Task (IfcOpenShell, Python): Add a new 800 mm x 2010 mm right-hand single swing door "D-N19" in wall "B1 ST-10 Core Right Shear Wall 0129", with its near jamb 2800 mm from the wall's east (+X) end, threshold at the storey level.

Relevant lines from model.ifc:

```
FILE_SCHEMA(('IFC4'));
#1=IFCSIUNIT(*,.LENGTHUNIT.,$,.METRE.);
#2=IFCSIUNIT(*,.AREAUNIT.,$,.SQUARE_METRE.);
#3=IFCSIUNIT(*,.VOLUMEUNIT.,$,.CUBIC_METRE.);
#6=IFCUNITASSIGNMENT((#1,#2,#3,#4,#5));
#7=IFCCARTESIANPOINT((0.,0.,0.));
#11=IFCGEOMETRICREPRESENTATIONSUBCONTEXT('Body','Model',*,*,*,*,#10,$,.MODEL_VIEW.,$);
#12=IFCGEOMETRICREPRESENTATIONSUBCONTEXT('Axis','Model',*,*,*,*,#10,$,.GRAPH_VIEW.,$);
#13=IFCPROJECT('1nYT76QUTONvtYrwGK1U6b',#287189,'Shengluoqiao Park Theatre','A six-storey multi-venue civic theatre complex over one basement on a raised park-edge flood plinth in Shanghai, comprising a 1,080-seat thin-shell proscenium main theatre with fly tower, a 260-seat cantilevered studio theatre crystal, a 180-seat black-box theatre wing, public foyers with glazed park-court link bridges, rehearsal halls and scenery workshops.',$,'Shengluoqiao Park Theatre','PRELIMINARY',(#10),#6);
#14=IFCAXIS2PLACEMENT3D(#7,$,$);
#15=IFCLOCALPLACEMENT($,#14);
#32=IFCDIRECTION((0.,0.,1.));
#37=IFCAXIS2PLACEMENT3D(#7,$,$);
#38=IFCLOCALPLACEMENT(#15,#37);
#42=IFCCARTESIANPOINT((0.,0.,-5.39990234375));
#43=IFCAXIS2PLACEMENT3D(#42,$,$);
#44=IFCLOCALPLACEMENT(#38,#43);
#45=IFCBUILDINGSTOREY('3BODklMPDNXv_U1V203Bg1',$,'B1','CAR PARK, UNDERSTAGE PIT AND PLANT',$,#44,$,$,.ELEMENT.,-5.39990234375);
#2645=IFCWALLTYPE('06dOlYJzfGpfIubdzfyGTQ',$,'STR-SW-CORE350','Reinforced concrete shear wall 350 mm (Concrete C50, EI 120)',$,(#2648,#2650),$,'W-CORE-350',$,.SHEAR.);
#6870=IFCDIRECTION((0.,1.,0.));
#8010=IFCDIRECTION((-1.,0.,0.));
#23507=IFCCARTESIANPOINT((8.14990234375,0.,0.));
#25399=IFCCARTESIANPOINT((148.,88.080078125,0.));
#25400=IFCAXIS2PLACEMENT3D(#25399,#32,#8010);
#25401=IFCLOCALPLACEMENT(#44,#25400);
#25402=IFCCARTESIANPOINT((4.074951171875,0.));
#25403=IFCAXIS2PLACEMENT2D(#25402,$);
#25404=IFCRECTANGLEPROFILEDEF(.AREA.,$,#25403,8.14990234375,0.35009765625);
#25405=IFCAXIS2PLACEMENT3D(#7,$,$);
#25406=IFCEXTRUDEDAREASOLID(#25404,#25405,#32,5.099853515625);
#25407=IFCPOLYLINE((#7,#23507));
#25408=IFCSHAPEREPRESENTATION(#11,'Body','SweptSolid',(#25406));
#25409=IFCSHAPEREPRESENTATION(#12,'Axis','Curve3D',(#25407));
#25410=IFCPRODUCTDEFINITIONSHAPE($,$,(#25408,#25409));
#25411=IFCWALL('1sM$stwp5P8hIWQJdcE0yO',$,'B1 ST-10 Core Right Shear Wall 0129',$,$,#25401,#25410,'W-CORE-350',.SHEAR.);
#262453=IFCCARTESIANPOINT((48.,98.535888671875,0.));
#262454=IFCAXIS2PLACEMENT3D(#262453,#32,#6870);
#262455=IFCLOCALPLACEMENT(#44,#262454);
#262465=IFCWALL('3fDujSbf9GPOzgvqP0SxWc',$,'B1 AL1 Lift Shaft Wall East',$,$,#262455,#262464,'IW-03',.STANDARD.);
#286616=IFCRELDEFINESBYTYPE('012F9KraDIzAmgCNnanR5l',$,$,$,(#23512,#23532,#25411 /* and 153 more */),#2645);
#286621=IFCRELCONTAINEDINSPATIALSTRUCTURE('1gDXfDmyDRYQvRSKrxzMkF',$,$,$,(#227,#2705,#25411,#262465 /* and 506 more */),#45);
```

```python
import numpy as np
import ifcopenshell
import ifcopenshell.api.feature
import ifcopenshell.api.geometry
import ifcopenshell.api.root
import ifcopenshell.api.spatial
import ifcopenshell.geom
import ifcopenshell.util.element
import ifcopenshell.util.placement
import ifcopenshell.util.representation
import ifcopenshell.util.shape
import ifcopenshell.util.unit

model = ifcopenshell.open("model.ifc")
unit_scale = ifcopenshell.util.unit.calculate_unit_scale(model)
settings = ifcopenshell.geom.settings()


def volume(element):
    """Net volume in cubic metres, openings subtracted."""
    shape = ifcopenshell.geom.create_shape(settings, element)
    return ifcopenshell.util.shape.get_volume(shape.geometry)


wall = model.by_guid("1sM$stwp5P8hIWQJdcE0yO")
storey = ifcopenshell.util.element.get_container(wall, ifc_class="IfcBuildingStorey")
context = ifcopenshell.util.representation.get_context(model, "Model", "Body", "MODEL_VIEW")
before = volume(wall)

width, height, from_end, sill = 0.8, 2.01, 2.8, 0.0  # metres

# The wall runs along its own X axis, and the end named is its -X end.
wall_shape = ifcopenshell.geom.create_shape(settings, wall)
x, y, z = ifcopenshell.util.shape.get_vertices(wall_shape.geometry).T
start = x.min() + from_end
face, thickness = float(y.min()), float(y.max() - y.min())
wall_matrix = ifcopenshell.util.placement.get_local_placement(wall.ObjectPlacement)
level = ifcopenshell.util.placement.get_local_placement(storey.ObjectPlacement)[2, 3]


def in_wall(x, y):
    """Placement at x, y metres in the wall's axes, at sill height."""
    matrix = wall_matrix.copy()
    matrix[:, 3] = wall_matrix @ np.array([x / unit_scale, y / unit_scale, 0.0, 1.0])
    matrix[2, 3] = level + sill / unit_scale
    return matrix


# Opening: a box that overshoots both wall faces by 50 mm.
opening = ifcopenshell.api.root.create_entity(model, ifc_class="IfcOpeningElement", predefined_type="OPENING")
box = ifcopenshell.api.geometry.add_wall_representation(
    model, context=context, length=width, height=height, thickness=thickness + 0.1
)
ifcopenshell.api.geometry.assign_representation(model, product=opening, representation=box)
ifcopenshell.api.geometry.edit_object_placement(model, product=opening, matrix=in_wall(start, face - 0.05), is_si=False)
ifcopenshell.api.feature.add_feature(model, feature=opening, element=wall)

door = ifcopenshell.api.root.create_entity(model, ifc_class="IfcDoor", name="D-N19", predefined_type="DOOR")
door.OverallWidth, door.OverallHeight = width / unit_scale, height / unit_scale
door.OperationType = "SINGLE_SWING_RIGHT"
body = ifcopenshell.api.geometry.add_door_representation(
    model,
    context=context,
    overall_width=door.OverallWidth,
    overall_height=door.OverallHeight,
    operation_type="SINGLE_SWING_RIGHT",
    lining_properties={"LiningDepth": thickness / unit_scale, "ThresholdDepth": thickness / unit_scale},
)
ifcopenshell.api.geometry.assign_representation(model, product=door, representation=body)
ifcopenshell.api.spatial.assign_container(model, products=[door], relating_structure=storey)
ifcopenshell.api.feature.add_filling(model, opening=opening, element=door)

# The lining spans the wall, so the door starts at the wall face.
ifcopenshell.api.geometry.edit_object_placement(model, product=door, matrix=in_wall(start, face), is_si=False)

after = volume(wall)

print(f"wall volume {before:.3f} -> {after:.3f} m3")

model.write("model_v2.ifc")
```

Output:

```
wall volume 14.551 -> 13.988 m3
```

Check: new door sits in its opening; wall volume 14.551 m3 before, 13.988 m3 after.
